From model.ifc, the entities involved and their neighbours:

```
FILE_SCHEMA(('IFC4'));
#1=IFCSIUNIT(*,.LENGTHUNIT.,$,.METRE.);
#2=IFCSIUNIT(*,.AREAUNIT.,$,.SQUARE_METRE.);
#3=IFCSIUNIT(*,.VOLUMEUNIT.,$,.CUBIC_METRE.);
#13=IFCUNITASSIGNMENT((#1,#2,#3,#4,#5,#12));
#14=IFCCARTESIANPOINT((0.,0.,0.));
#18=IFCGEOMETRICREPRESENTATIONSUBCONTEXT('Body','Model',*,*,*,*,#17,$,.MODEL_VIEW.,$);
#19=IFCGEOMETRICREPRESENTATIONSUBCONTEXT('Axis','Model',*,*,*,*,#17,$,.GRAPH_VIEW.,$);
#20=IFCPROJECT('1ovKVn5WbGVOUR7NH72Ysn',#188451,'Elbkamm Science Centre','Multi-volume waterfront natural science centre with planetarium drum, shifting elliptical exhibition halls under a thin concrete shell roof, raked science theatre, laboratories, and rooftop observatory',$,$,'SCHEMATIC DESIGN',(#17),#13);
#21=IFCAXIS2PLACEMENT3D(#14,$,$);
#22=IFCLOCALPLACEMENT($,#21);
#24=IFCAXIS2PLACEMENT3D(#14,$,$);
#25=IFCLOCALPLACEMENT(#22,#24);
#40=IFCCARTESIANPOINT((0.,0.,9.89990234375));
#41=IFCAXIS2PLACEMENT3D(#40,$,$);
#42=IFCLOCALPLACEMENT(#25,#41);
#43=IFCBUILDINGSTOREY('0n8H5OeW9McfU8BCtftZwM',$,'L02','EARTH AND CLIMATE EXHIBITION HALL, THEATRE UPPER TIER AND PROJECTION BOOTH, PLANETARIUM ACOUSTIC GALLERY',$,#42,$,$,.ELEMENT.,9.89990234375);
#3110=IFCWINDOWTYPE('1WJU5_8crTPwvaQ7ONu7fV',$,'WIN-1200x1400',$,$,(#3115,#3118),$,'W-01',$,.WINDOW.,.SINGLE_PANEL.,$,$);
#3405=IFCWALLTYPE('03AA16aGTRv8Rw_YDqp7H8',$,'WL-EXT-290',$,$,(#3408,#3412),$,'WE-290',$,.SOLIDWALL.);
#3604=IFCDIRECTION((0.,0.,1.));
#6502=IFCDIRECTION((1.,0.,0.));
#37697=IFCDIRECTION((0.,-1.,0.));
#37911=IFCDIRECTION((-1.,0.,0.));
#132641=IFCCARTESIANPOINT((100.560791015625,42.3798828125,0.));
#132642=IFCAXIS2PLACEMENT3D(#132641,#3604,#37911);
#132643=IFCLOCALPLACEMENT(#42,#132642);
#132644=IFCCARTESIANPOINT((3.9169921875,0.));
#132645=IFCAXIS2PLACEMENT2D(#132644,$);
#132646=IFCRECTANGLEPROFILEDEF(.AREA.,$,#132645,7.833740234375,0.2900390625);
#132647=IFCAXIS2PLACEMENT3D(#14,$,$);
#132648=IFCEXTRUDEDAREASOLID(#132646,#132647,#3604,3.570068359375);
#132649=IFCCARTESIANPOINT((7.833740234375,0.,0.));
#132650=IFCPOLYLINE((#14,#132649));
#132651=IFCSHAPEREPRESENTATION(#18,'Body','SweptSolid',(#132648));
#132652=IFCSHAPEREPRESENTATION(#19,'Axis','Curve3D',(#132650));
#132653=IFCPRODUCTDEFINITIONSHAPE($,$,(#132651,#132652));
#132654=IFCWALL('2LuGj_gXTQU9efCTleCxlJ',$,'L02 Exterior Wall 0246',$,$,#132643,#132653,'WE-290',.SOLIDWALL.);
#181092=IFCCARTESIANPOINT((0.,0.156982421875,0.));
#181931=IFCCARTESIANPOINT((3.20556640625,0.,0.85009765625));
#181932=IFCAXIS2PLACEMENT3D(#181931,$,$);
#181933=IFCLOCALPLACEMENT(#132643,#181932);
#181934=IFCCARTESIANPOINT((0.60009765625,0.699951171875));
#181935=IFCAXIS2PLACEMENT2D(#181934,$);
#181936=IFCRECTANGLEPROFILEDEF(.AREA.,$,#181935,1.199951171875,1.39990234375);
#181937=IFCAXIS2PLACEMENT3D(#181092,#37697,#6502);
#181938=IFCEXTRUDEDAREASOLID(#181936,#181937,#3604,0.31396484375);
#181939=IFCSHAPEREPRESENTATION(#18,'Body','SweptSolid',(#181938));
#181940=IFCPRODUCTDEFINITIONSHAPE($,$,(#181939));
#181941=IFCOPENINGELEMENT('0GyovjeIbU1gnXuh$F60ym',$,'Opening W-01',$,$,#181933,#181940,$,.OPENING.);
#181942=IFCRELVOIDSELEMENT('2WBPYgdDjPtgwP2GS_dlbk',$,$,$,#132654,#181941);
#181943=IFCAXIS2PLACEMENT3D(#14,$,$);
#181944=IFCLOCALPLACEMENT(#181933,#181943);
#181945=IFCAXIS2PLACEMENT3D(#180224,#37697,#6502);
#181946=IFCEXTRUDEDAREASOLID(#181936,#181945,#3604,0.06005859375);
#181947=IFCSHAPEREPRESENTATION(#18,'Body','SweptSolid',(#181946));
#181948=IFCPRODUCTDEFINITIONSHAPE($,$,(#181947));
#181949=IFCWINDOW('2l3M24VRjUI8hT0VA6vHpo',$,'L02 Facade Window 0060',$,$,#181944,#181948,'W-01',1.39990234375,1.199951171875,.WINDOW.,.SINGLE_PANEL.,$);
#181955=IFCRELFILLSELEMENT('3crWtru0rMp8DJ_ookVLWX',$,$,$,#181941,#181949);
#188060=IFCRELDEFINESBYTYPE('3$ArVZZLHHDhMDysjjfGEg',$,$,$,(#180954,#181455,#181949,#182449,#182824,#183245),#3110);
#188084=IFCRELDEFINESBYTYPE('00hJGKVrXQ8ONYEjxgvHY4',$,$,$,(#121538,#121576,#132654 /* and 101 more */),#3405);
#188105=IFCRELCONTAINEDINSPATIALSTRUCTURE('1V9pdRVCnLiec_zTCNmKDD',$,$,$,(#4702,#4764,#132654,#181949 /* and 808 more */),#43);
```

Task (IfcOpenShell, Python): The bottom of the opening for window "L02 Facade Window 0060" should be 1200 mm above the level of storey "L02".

```python
import numpy as np
import ifcopenshell
import ifcopenshell.api.geometry
import ifcopenshell.geom
import ifcopenshell.util.element
import ifcopenshell.util.placement
import ifcopenshell.util.shape
import ifcopenshell.util.unit

model = ifcopenshell.open("model.ifc")
unit_scale = ifcopenshell.util.unit.calculate_unit_scale(model)

window = model.by_guid("2l3M24VRjUI8hT0VA6vHpo")
opening = window.FillsVoids[0].RelatingOpeningElement
storey = ifcopenshell.util.element.get_container(window, ifc_class="IfcBuildingStorey")
level = ifcopenshell.util.placement.get_local_placement(storey.ObjectPlacement)[2, 3]

# The opening's origin need not be at the sill, so measure its lowest point.
shape = ifcopenshell.geom.create_shape(ifcopenshell.geom.settings(), opening)
bottom = ifcopenshell.util.shape.get_shape_bottom_elevation(shape, shape.geometry) / unit_scale
dz = level + 1.2 / unit_scale - bottom

shift = np.array([0.0, 0.0, dz])
# The window is placed relative to its opening, so it follows when the opening moves.
matrix = ifcopenshell.util.placement.get_local_placement(opening.ObjectPlacement)
matrix[:3, 3] += shift
ifcopenshell.api.geometry.edit_object_placement(
    model, product=opening, matrix=matrix, is_si=False, should_transform_children=True
)

print(f"moved by {dz * unit_scale:+.3f} m")

model.write("model_v2.ifc")
```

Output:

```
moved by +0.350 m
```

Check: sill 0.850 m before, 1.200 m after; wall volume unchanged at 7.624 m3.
